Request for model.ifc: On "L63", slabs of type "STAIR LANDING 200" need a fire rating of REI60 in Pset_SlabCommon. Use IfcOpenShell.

First a look at what the model holds.

```python
import ifcopenshell
import ifcopenshell.util.element

model = ifcopenshell.open("model.ifc")
print(model.schema)
storey = next(s for s in model.by_type("IfcBuildingStorey") if s.Name == "L63")
slabs = [e for e in ifcopenshell.util.element.get_decomposition(storey) if e.is_a("IfcSlab")]
seen = {}
for e in slabs:
    element_type = ifcopenshell.util.element.get_type(e)
    key = (element_type.Name if element_type != e and element_type else None, ifcopenshell.util.element.get_pset(e, "Pset_SlabCommon", "FireRating"))
    seen[key] = seen.get(key, 0) + 1
for (name, value), count in sorted(seen.items(), key=str):
    print(count, "x", name, "|", value)
```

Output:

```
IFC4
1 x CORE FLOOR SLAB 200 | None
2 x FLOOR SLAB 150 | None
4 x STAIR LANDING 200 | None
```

```python
import ifcopenshell
import ifcopenshell.api.pset
import ifcopenshell.util.element

model = ifcopenshell.open("model.ifc")

storey = next(s for s in model.by_type("IfcBuildingStorey") if s.Name == "L63")
slabs = [e for e in ifcopenshell.util.element.get_decomposition(storey) if e.is_a("IfcSlab")]

count = 0
for e in slabs:
    element_type = ifcopenshell.util.element.get_type(e)
    if element_type in (None, e) or element_type.Name != "STAIR LANDING 200":
        continue
    found = ifcopenshell.util.element.get_pset(e, "Pset_SlabCommon", should_inherit=False)
    if found:
        pset = model.by_id(found["id"])
        if len(ifcopenshell.util.element.get_elements_by_pset(pset)) > 1:
            pset = ifcopenshell.api.pset.unshare_pset(model, products=[e], pset=pset)[0]
    else:
        pset = ifcopenshell.api.pset.add_pset(model, product=e, name="Pset_SlabCommon")
    ifcopenshell.api.pset.edit_pset(model, pset=pset, properties={"FireRating": "REI60"})
    count += 1

print(count, "slabs updated")

model.write("model_rev.ifc")
```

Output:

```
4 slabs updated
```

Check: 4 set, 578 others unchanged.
